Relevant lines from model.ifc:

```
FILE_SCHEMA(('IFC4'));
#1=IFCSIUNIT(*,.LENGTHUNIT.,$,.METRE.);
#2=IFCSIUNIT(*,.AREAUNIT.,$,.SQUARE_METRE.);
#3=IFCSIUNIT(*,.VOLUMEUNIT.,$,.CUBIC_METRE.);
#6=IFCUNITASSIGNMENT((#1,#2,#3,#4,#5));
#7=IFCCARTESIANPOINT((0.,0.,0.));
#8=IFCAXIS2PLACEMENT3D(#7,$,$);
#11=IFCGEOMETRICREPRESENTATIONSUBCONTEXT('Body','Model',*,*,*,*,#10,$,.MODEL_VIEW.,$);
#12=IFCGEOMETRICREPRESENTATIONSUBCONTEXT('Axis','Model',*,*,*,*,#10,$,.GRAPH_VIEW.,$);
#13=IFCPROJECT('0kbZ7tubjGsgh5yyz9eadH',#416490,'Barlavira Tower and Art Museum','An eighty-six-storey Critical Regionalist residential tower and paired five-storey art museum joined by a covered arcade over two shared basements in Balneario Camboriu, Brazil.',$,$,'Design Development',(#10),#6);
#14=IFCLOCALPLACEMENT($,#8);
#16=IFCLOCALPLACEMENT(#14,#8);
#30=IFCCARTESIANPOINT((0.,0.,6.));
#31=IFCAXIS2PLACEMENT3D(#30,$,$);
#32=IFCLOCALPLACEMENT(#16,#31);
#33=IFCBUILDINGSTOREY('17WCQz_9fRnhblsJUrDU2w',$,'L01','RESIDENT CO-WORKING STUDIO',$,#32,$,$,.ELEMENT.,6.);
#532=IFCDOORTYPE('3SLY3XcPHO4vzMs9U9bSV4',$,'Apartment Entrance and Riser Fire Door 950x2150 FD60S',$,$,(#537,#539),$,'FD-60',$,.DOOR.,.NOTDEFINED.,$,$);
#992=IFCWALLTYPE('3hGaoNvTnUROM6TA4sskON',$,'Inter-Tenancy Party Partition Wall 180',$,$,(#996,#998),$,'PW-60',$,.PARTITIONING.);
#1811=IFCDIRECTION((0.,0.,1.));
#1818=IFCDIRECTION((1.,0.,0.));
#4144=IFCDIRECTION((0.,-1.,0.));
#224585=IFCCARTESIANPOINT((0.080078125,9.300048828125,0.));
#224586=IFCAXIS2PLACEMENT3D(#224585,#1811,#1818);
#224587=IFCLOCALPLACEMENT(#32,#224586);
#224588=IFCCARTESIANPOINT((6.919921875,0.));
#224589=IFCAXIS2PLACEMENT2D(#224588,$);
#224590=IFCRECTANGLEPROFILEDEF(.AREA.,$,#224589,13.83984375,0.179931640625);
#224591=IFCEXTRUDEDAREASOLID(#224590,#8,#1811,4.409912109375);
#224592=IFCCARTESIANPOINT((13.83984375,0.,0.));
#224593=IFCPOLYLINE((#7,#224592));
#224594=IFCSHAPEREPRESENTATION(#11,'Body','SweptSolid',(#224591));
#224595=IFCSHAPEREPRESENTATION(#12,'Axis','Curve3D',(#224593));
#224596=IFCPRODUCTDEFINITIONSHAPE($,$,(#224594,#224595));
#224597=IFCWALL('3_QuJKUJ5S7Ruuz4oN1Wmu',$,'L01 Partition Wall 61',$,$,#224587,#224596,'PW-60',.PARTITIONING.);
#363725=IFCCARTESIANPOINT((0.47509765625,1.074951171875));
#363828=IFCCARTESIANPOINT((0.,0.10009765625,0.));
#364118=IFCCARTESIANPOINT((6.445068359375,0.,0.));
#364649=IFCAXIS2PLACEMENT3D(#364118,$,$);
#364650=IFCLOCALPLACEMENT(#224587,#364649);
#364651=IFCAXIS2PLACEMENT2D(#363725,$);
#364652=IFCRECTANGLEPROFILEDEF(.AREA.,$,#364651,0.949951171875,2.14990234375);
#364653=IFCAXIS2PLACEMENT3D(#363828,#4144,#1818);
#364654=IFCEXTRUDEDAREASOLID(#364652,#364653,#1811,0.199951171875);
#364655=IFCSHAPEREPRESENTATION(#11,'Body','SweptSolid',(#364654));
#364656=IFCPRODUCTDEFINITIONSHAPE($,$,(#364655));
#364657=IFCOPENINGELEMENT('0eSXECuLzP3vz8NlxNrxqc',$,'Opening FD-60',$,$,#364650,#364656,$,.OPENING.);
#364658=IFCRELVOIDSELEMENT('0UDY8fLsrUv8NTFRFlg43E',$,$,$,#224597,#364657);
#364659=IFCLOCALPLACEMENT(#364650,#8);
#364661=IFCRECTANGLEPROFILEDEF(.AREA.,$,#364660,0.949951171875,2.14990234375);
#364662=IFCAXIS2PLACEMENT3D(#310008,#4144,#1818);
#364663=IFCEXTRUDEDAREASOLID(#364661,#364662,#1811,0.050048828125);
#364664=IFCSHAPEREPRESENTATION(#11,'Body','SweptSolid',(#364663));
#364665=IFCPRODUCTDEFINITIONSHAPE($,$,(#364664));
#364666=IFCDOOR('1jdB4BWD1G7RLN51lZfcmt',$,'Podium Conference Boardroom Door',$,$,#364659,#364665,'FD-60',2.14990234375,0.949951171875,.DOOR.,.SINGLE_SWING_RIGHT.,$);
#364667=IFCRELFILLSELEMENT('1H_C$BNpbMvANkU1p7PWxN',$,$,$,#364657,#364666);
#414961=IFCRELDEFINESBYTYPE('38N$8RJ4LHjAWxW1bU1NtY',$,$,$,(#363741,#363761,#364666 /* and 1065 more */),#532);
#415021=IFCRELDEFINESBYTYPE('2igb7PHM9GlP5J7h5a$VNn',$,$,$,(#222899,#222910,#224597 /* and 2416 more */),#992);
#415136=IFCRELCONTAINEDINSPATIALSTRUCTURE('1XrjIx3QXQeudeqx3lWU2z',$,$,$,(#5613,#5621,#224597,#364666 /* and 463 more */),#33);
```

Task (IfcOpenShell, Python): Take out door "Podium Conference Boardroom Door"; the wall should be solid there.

```python
import ifcopenshell
import ifcopenshell.api.feature
import ifcopenshell.api.root
import ifcopenshell.geom
import ifcopenshell.util.shape

model = ifcopenshell.open("model.ifc")
settings = ifcopenshell.geom.settings()


def volume(element):
    """Net volume in cubic metres, openings subtracted."""
    shape = ifcopenshell.geom.create_shape(settings, element)
    return ifcopenshell.util.shape.get_volume(shape.geometry)


door = model.by_id(364666)
opening = door.FillsVoids[0].RelatingOpeningElement
wall = opening.VoidsElements[0].RelatingBuildingElement
before = volume(wall)

ifcopenshell.api.root.remove_product(model, product=door)
ifcopenshell.api.feature.remove_feature(model, feature=opening)

after = volume(wall)

print(f"wall volume {before:.3f} -> {after:.3f} m3")

model.write("model_v2.ifc")
```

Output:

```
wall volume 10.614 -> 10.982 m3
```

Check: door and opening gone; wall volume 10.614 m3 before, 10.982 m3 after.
